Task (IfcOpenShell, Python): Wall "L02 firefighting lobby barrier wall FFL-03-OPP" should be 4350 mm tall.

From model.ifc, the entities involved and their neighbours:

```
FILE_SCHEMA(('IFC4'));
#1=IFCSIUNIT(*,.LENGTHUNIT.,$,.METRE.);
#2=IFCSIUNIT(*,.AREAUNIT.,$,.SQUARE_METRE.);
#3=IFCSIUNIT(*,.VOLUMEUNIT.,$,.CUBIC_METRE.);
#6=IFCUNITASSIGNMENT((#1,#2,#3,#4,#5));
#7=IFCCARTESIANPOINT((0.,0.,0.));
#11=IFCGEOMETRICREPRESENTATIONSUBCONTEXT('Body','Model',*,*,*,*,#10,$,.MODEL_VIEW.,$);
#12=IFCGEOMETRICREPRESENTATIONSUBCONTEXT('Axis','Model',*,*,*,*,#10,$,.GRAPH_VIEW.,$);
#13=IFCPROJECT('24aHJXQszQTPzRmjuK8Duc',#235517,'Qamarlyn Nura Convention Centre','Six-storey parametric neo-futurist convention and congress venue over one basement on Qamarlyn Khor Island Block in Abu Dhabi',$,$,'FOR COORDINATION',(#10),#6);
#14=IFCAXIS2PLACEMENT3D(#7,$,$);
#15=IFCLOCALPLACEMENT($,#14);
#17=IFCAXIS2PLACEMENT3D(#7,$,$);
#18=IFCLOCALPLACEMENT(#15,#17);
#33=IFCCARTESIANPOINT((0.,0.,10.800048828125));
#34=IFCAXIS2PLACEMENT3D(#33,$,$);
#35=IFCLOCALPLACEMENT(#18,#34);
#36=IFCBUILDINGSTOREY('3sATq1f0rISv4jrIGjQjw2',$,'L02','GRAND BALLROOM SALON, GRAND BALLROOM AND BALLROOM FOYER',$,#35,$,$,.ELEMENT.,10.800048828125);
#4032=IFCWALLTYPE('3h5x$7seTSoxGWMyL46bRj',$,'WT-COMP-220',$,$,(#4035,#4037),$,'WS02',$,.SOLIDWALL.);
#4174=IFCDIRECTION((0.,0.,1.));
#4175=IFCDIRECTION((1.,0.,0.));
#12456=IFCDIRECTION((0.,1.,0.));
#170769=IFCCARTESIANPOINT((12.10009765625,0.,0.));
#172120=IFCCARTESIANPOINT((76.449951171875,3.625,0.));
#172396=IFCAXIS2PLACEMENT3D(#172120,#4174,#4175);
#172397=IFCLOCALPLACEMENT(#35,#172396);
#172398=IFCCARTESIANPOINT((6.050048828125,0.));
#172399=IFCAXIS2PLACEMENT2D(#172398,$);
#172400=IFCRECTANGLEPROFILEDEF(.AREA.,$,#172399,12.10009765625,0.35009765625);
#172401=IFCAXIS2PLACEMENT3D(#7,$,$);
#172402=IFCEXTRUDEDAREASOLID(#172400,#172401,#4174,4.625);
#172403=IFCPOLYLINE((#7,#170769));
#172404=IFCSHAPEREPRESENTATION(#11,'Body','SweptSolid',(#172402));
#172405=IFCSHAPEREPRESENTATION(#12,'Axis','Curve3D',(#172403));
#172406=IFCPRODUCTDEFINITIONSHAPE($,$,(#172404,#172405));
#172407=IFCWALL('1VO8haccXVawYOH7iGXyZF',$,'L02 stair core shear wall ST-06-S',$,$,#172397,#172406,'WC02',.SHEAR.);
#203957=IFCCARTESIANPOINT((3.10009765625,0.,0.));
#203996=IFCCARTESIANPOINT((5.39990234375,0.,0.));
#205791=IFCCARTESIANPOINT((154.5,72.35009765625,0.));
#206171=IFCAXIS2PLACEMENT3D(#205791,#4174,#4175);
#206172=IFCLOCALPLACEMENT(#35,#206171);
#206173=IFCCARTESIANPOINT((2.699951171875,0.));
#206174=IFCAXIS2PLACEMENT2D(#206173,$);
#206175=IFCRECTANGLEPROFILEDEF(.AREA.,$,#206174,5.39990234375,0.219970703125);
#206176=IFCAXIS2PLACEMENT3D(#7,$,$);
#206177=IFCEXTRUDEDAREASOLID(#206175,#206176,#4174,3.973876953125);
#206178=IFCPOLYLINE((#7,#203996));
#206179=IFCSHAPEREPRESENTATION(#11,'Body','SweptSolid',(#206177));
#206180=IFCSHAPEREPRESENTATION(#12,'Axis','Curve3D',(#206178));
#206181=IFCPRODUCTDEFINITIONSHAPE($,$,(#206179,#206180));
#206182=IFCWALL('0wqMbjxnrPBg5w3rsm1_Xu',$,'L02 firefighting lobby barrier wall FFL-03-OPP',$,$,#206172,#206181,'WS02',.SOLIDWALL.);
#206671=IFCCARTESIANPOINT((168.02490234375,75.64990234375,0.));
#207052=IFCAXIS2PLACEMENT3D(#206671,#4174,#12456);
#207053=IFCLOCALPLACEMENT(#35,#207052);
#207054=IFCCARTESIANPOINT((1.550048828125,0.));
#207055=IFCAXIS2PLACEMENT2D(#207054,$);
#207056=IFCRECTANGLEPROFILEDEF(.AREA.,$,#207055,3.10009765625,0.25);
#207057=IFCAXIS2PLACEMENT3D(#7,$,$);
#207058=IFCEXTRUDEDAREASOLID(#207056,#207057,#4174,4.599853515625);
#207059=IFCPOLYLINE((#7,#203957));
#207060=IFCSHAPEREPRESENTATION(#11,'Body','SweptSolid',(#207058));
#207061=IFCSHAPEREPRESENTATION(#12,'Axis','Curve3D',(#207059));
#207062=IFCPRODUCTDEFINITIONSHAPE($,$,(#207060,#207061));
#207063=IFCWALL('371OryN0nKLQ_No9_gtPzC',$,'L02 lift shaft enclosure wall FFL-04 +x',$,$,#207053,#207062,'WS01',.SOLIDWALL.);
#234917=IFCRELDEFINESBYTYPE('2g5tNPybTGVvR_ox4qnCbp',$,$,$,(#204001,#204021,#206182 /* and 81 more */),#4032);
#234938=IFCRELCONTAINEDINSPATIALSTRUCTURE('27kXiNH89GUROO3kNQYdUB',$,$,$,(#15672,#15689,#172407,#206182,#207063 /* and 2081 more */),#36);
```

```python
import ifcopenshell
import ifcopenshell.geom
import ifcopenshell.util.representation
import ifcopenshell.util.shape
import ifcopenshell.util.unit

model = ifcopenshell.open("model.ifc")
unit_scale = ifcopenshell.util.unit.calculate_unit_scale(model)
settings = ifcopenshell.geom.settings()


def volume(element):
    """Net volume in cubic metres, openings subtracted."""
    shape = ifcopenshell.geom.create_shape(settings, element)
    return ifcopenshell.util.shape.get_volume(shape.geometry)


wall = model.by_guid("0wqMbjxnrPBg5w3rsm1_Xu")
before = volume(wall)

body = ifcopenshell.util.representation.get_representation(wall, "Model", "Body")
solid = body.Items[0]
old_height = solid.Depth
solid.Depth = 4.35 / unit_scale
after = volume(wall)

print(f"height {old_height:g} -> {solid.Depth:g}, volume {before:.3f} -> {after:.3f} m3")

model.write("model_edited.ifc")
```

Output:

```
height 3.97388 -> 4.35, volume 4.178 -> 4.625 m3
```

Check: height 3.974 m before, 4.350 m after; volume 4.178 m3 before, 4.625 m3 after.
